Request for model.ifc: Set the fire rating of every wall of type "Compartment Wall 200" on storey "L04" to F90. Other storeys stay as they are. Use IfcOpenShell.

First a look at what the model holds.

```python
import ifcopenshell
import ifcopenshell.util.element

model = ifcopenshell.open("model.ifc")
print(model.schema)
storey = next(s for s in model.by_type("IfcBuildingStorey") if s.Name == "L04")
walls = [e for e in ifcopenshell.util.element.get_decomposition(storey) if e.is_a("IfcWall")]
seen = {}
for e in walls:
    element_type = ifcopenshell.util.element.get_type(e)
    key = (element_type.Name if element_type != e and element_type else None, ifcopenshell.util.element.get_pset(e, "Pset_WallCommon", "FireRating"))
    seen[key] = seen.get(key, 0) + 1
for (name, value), count in sorted(seen.items(), key=str):
    print(count, "x", name, "|", value)
```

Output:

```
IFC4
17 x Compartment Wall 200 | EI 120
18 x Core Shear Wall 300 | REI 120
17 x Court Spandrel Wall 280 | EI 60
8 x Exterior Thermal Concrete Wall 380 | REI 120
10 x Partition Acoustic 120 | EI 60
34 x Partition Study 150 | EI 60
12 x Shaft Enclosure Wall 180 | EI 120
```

```python
import ifcopenshell
import ifcopenshell.api.pset
import ifcopenshell.util.element

model = ifcopenshell.open("model.ifc")

storey = next(s for s in model.by_type("IfcBuildingStorey") if s.Name == "L04")
walls = [e for e in ifcopenshell.util.element.get_decomposition(storey) if e.is_a("IfcWall")]

count = 0
for e in walls:
    element_type = ifcopenshell.util.element.get_type(e)
    if element_type in (None, e) or element_type.Name != "Compartment Wall 200":
        continue
    # add_pset returns the element's existing set when there is one.
    pset = ifcopenshell.api.pset.add_pset(model, product=e, name="Pset_WallCommon")
    ifcopenshell.api.pset.edit_pset(model, pset=pset, properties={"FireRating": "F90"})
    count += 1

print(count, "walls updated")

model.write("model_updated.ifc")
```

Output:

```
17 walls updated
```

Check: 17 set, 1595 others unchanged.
